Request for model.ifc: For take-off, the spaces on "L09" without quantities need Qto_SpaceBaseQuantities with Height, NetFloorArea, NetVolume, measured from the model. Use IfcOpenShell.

First a look at what the model holds.

```python
import ifcopenshell
import ifcopenshell.util.element
import ifcopenshell.util.unit

model = ifcopenshell.open("model.ifc")
print(model.schema)
for unit_type in ("LENGTHUNIT", "AREAUNIT", "VOLUMEUNIT"):
    print(unit_type, ifcopenshell.util.unit.calculate_unit_scale(model, unit_type))
storey = next(s for s in model.by_type("IfcBuildingStorey") if s.Name == "L09")
spaces = [e for e in ifcopenshell.util.element.get_decomposition(storey) if e.is_a("IfcSpace")]
for e in sorted(spaces, key=lambda e: e.id()):
    print(e.id(), e.is_a(), e.Name, list(ifcopenshell.util.element.get_psets(e, qtos_only=True)), sep=" | ")
```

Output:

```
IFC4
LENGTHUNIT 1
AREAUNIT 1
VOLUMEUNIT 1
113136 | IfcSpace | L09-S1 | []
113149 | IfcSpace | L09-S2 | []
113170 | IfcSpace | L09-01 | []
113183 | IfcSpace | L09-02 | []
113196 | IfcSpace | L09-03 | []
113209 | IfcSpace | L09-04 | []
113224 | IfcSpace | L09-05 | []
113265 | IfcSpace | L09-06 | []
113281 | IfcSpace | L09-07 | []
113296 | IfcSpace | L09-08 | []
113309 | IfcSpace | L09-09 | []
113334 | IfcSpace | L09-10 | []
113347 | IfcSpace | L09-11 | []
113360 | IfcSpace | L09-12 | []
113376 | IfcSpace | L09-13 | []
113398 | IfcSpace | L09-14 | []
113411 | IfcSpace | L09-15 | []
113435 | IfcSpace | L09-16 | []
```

```python
import ifcopenshell
import ifcopenshell.api.pset
import ifcopenshell.geom
import ifcopenshell.util.element
import ifcopenshell.util.shape
import ifcopenshell.util.unit

model = ifcopenshell.open("model.ifc")
unit_scale = ifcopenshell.util.unit.calculate_unit_scale(model)
area_scale = ifcopenshell.util.unit.calculate_unit_scale(model, "AREAUNIT")
volume_scale = ifcopenshell.util.unit.calculate_unit_scale(model, "VOLUMEUNIT")
settings = ifcopenshell.geom.settings()

storey = next(s for s in model.by_type("IfcBuildingStorey") if s.Name == "L09")
spaces = [e for e in ifcopenshell.util.element.get_decomposition(storey) if e.is_a("IfcSpace")]

for e in sorted(spaces, key=lambda e: e.id()):
    if ifcopenshell.util.element.get_psets(e, qtos_only=True, should_inherit=False):
        continue
    # Geometry comes back in metres, in the element's own axes.
    shape = ifcopenshell.geom.create_shape(settings, e)
    values = {
        "Height": ifcopenshell.util.shape.get_z(shape.geometry) / unit_scale,
        "NetFloorArea": ifcopenshell.util.shape.get_footprint_area(shape.geometry) / area_scale,
        "NetVolume": ifcopenshell.util.shape.get_volume(shape.geometry) / volume_scale,
    }
    qto = ifcopenshell.api.pset.add_qto(model, product=e, name="Qto_SpaceBaseQuantities")
    ifcopenshell.api.pset.edit_qto(model, qto=qto, properties=values)
    print(e.id(), {k: round(v, 3) for k, v in values.items()})

model.write("model_v2.ifc")
```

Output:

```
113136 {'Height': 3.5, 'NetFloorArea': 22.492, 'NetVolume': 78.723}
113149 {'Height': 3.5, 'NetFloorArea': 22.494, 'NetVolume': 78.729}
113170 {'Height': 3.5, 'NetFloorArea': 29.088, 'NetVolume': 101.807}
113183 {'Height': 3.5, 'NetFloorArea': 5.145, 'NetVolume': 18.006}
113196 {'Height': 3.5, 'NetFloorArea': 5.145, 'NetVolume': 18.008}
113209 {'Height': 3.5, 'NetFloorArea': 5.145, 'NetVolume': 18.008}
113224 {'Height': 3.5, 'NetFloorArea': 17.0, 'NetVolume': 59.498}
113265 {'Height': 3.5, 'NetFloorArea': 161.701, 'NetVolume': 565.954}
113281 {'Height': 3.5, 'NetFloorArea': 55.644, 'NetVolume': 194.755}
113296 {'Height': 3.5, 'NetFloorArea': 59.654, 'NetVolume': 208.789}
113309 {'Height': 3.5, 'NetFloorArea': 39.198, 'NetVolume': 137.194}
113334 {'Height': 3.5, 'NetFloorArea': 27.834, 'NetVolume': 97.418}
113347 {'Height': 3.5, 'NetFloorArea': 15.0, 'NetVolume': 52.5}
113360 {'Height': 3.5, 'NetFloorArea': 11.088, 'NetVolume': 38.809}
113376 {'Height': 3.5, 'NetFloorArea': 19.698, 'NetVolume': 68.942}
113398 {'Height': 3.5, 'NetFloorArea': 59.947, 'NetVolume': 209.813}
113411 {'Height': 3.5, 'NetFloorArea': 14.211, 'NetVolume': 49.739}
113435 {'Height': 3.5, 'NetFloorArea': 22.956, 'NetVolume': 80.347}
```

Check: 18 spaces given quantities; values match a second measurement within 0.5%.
